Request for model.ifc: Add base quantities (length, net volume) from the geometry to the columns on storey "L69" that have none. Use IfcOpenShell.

First a look at what the model holds.

```python
import ifcopenshell
import ifcopenshell.util.element
import ifcopenshell.util.unit

model = ifcopenshell.open("model.ifc")
print(model.schema)
for unit_type in ("LENGTHUNIT", "AREAUNIT", "VOLUMEUNIT"):
    print(unit_type, ifcopenshell.util.unit.calculate_unit_scale(model, unit_type))
storey = next(s for s in model.by_type("IfcBuildingStorey") if s.Name == "L69")
columns = [e for e in ifcopenshell.util.element.get_decomposition(storey) if e.is_a("IfcColumn")]
for e in sorted(columns, key=lambda e: e.id()):
    print(e.id(), e.is_a(), e.Name, list(ifcopenshell.util.element.get_psets(e, qtos_only=True)), sep=" | ")
```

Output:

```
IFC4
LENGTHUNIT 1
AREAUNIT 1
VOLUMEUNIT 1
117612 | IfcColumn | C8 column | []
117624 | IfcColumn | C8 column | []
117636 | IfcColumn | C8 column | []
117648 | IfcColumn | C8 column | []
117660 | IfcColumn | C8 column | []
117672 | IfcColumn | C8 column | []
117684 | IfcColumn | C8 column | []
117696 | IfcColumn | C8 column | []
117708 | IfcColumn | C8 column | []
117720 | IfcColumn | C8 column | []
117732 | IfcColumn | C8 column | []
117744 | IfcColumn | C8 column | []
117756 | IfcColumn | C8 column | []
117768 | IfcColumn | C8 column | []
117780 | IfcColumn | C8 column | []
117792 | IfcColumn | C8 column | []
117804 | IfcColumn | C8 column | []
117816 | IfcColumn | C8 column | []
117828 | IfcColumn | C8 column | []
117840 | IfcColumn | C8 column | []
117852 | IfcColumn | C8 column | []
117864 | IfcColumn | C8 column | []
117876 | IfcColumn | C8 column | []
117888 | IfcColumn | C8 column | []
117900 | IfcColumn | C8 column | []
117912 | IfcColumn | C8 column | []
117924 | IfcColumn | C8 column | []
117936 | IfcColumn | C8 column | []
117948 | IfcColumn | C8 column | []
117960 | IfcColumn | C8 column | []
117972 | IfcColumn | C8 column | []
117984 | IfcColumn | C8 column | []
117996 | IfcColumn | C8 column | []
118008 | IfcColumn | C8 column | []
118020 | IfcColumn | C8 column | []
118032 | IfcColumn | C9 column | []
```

```python
import ifcopenshell
import ifcopenshell.api.pset
import ifcopenshell.geom
import ifcopenshell.util.element
import ifcopenshell.util.shape
import ifcopenshell.util.unit

model = ifcopenshell.open("model.ifc")
unit_scale = ifcopenshell.util.unit.calculate_unit_scale(model)
volume_scale = ifcopenshell.util.unit.calculate_unit_scale(model, "VOLUMEUNIT")
settings = ifcopenshell.geom.settings()

storey = next(s for s in model.by_type("IfcBuildingStorey") if s.Name == "L69")
columns = [e for e in ifcopenshell.util.element.get_decomposition(storey) if e.is_a("IfcColumn")]

for e in sorted(columns, key=lambda e: e.id()):
    if ifcopenshell.util.element.get_psets(e, qtos_only=True, should_inherit=False):
        continue
    # Geometry comes back in metres, in the element's own axes.
    shape = ifcopenshell.geom.create_shape(settings, e)
    values = {
        "Length": ifcopenshell.util.shape.get_z(shape.geometry) / unit_scale,
        "NetVolume": ifcopenshell.util.shape.get_volume(shape.geometry) / volume_scale,
    }
    qto = ifcopenshell.api.pset.add_qto(model, product=e, name="Qto_ColumnBaseQuantities")
    ifcopenshell.api.pset.edit_qto(model, qto=qto, properties=values)
    print(e.id(), {k: round(v, 3) for k, v in values.items()})

model.write("model_updated.ifc")
```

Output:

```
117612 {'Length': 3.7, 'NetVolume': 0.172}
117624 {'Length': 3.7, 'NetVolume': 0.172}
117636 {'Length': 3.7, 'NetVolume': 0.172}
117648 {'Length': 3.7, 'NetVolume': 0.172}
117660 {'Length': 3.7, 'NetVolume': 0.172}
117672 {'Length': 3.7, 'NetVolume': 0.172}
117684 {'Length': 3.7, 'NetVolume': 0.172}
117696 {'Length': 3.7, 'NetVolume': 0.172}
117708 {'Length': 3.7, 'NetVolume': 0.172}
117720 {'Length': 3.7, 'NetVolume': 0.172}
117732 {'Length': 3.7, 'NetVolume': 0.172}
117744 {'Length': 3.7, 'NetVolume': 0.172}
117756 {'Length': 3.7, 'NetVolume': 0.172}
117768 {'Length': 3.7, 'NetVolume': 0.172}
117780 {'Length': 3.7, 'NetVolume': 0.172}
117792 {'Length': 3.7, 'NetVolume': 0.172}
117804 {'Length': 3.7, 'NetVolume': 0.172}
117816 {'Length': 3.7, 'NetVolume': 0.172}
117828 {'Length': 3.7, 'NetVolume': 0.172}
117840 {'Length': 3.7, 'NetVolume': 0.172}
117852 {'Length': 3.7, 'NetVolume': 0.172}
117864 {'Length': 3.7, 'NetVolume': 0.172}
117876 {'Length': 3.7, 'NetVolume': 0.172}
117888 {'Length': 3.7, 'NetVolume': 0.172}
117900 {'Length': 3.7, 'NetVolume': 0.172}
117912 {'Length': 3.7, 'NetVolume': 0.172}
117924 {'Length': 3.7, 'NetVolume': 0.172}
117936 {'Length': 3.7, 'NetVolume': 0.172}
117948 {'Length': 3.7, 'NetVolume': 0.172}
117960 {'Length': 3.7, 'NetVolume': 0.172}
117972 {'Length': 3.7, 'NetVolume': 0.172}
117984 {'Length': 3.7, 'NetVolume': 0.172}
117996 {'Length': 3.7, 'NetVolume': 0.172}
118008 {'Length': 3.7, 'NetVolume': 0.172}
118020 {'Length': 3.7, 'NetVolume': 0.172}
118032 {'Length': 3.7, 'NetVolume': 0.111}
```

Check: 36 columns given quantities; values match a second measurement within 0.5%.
